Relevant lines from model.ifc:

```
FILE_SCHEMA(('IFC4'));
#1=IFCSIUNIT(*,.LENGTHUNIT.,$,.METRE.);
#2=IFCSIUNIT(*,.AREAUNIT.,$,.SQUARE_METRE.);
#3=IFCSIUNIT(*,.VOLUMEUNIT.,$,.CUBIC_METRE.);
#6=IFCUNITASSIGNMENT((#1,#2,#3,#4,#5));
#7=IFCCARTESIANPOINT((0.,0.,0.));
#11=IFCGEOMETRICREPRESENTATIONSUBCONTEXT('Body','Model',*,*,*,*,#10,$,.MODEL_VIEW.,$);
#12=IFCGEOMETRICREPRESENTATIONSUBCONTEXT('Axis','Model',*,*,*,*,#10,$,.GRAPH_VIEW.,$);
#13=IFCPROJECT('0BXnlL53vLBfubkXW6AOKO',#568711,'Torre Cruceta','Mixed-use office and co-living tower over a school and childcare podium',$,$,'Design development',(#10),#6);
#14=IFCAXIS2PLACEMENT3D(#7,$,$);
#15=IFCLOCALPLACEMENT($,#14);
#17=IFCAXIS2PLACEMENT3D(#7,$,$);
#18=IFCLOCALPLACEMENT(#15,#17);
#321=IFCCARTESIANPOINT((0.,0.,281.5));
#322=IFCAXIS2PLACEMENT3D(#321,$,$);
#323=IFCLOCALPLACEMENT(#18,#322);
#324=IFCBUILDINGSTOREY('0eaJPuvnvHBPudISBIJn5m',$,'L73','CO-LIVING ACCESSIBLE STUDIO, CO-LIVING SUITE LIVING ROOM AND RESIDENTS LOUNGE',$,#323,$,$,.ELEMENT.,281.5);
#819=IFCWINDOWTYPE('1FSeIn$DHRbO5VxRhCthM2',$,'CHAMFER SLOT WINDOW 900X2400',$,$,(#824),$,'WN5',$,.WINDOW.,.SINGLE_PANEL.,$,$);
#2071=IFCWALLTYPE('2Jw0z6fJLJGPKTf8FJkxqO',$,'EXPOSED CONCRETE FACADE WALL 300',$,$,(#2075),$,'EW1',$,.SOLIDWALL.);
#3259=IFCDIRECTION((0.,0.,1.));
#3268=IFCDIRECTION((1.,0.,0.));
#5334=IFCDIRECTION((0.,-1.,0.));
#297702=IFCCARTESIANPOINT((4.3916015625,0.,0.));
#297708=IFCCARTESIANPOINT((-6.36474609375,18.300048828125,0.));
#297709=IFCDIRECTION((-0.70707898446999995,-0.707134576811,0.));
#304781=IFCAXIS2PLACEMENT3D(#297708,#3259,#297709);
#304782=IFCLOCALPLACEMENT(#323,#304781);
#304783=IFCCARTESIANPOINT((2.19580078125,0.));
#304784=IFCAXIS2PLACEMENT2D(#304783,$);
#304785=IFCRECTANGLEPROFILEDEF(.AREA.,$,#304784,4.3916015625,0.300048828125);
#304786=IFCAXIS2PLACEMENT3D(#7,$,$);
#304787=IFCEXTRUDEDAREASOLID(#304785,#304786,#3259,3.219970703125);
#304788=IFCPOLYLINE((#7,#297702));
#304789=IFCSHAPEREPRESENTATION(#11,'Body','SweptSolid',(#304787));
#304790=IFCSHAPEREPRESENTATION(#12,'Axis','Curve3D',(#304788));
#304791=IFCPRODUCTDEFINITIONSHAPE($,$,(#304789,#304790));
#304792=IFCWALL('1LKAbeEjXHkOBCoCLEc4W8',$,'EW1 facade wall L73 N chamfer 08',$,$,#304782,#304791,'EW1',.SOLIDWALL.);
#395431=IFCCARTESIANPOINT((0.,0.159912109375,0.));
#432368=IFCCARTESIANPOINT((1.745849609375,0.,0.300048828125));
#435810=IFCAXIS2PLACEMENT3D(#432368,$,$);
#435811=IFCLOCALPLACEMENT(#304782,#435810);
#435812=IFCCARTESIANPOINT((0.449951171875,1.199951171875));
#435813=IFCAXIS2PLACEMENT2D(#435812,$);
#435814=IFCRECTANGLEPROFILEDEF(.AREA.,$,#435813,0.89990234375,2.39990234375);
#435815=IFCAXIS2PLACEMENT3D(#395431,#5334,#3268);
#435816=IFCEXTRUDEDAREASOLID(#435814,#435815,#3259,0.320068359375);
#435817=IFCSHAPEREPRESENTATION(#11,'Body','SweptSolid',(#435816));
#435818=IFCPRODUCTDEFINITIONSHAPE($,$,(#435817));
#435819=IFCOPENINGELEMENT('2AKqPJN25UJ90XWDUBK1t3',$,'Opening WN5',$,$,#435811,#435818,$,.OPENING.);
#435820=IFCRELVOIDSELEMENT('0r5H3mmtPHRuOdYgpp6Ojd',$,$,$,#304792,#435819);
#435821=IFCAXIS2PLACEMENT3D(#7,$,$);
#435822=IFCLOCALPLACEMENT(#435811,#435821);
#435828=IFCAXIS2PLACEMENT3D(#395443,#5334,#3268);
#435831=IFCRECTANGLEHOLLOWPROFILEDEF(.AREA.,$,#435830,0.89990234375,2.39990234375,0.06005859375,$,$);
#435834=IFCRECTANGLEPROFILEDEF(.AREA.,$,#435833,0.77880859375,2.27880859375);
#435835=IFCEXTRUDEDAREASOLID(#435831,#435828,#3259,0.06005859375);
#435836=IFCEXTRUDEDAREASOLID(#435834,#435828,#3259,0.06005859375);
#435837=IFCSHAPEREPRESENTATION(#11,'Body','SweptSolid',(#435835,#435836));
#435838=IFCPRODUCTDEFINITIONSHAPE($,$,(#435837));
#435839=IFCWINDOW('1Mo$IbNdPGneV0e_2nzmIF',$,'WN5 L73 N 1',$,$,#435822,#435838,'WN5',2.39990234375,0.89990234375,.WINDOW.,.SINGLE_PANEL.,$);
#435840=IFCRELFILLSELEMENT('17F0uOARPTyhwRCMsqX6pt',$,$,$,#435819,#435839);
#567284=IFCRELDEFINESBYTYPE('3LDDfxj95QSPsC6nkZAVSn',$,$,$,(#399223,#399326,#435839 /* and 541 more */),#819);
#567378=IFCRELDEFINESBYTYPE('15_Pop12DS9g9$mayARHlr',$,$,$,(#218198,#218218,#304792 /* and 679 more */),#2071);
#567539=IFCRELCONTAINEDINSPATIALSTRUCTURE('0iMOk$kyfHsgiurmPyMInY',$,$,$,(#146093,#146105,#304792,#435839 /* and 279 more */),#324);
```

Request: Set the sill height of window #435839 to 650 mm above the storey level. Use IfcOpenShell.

```python
import numpy as np
import ifcopenshell
import ifcopenshell.api.geometry
import ifcopenshell.geom
import ifcopenshell.util.element
import ifcopenshell.util.placement
import ifcopenshell.util.shape
import ifcopenshell.util.unit

model = ifcopenshell.open("model.ifc")
unit_scale = ifcopenshell.util.unit.calculate_unit_scale(model)

window = model.by_guid("1Mo$IbNdPGneV0e_2nzmIF")
opening = window.FillsVoids[0].RelatingOpeningElement
storey = ifcopenshell.util.element.get_container(window, ifc_class="IfcBuildingStorey")
level = ifcopenshell.util.placement.get_local_placement(storey.ObjectPlacement)[2, 3]

# The opening's origin need not be at the sill, so measure its lowest point.
shape = ifcopenshell.geom.create_shape(ifcopenshell.geom.settings(), opening)
bottom = ifcopenshell.util.shape.get_shape_bottom_elevation(shape, shape.geometry) / unit_scale
dz = level + 0.65 / unit_scale - bottom

shift = np.array([0.0, 0.0, dz])
# The window is placed relative to its opening, so it follows when the opening moves.
matrix = ifcopenshell.util.placement.get_local_placement(opening.ObjectPlacement)
matrix[:3, 3] += shift
ifcopenshell.api.geometry.edit_object_placement(
    model, product=opening, matrix=matrix, is_si=False, should_transform_children=True
)

print(f"moved by {dz * unit_scale:+.3f} m")

model.write("model_rev.ifc")
```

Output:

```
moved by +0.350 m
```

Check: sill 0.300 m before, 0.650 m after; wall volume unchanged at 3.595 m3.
